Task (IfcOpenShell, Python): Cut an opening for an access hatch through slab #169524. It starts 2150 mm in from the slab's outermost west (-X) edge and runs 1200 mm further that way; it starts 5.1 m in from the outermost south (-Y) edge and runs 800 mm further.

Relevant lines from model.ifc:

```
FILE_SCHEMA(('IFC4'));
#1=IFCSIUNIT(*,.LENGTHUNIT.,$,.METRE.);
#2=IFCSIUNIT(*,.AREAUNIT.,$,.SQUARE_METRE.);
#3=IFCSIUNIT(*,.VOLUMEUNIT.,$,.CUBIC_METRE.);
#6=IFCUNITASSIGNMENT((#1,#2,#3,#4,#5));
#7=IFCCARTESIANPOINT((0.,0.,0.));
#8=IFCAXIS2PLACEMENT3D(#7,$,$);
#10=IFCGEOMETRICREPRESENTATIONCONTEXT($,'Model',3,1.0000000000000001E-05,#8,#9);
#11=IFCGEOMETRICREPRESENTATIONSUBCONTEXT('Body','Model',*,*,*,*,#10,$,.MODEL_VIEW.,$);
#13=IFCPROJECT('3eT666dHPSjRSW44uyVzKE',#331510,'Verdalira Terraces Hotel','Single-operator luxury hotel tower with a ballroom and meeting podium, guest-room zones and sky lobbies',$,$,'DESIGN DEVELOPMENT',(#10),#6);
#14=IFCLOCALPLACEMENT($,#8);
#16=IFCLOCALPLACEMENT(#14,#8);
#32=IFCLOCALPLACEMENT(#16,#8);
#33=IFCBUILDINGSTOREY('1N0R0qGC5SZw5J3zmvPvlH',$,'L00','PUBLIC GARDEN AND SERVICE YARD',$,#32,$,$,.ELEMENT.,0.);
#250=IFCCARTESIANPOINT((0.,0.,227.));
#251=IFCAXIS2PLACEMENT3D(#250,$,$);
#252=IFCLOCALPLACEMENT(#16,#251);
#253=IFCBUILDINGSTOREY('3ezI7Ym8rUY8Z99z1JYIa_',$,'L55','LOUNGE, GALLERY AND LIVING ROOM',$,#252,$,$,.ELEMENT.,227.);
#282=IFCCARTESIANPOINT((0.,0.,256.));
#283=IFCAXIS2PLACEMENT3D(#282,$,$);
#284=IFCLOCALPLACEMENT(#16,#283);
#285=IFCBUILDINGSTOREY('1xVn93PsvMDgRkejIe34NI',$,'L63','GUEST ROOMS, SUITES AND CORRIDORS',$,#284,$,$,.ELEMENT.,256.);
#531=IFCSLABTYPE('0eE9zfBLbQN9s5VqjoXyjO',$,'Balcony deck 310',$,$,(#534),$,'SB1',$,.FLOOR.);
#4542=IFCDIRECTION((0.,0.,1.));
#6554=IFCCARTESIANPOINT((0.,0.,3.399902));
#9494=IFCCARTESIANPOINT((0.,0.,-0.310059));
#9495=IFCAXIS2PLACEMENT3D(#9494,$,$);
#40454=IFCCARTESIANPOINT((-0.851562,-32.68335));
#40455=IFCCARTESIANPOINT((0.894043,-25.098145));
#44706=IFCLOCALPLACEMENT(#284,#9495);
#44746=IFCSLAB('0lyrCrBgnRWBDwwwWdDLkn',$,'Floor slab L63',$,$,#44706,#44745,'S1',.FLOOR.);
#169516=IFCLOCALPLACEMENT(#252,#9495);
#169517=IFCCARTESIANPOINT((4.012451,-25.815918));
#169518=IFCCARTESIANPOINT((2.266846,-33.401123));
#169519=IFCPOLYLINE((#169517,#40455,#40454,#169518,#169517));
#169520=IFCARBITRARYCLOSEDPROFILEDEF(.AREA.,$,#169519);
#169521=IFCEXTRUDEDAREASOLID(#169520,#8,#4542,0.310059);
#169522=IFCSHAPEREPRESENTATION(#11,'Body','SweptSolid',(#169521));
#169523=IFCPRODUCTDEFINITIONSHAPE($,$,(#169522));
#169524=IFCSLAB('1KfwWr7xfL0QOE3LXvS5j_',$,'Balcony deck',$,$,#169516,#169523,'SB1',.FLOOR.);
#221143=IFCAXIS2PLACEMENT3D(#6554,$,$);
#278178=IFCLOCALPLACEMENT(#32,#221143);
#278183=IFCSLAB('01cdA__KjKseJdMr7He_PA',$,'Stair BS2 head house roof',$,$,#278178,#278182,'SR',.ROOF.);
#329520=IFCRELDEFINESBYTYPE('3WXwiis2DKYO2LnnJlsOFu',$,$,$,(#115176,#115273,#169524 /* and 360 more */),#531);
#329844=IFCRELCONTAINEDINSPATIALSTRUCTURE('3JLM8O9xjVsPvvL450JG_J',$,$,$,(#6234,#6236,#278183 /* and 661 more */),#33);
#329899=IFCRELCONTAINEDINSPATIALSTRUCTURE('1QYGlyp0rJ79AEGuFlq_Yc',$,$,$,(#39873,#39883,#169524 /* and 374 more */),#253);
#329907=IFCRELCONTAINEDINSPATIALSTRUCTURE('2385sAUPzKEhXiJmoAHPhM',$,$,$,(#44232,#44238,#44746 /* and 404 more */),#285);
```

```python
import numpy as np
import ifcopenshell
import ifcopenshell.api.feature
import ifcopenshell.api.geometry
import ifcopenshell.api.root
import ifcopenshell.geom
import ifcopenshell.util.placement
import ifcopenshell.util.representation
import ifcopenshell.util.shape
import ifcopenshell.util.unit

model = ifcopenshell.open("model.ifc")
unit_scale = ifcopenshell.util.unit.calculate_unit_scale(model)
settings = ifcopenshell.geom.settings()


def volume(element):
    """Net volume in cubic metres, openings subtracted."""
    shape = ifcopenshell.geom.create_shape(settings, element)
    return ifcopenshell.util.shape.get_volume(shape.geometry)


slab = model.by_id(169524)
before = volume(slab)

# Extent in the slab's own axes, in metres. The edges named are its -X and -Y sides.
slab_shape = ifcopenshell.geom.create_shape(settings, slab)
vertices = ifcopenshell.util.shape.get_vertices(slab_shape.geometry)
x_min, y_min, bottom = vertices.min(axis=0)
top = vertices[:, 2].max()

opening = ifcopenshell.api.root.create_entity(model, ifc_class="IfcOpeningElement", name="Access hatch opening", predefined_type="OPENING")
context = ifcopenshell.util.representation.get_context(model, "Model", "Body", "MODEL_VIEW")
width, depth = 1.2, 0.8
outline = [(0.0, 0.0), (width, 0.0), (width, depth), (0.0, depth), (0.0, 0.0)]
# Overshoot both faces by 50 mm so the cut is clean.
shape = ifcopenshell.api.geometry.add_slab_representation(
    model, context=context, depth=top - bottom + 0.1, polyline=outline
)
ifcopenshell.api.geometry.assign_representation(model, product=opening, representation=shape)

matrix = ifcopenshell.util.placement.get_local_placement(slab.ObjectPlacement)
matrix[:, 3] = matrix @ np.append(np.array([x_min + 2.15, y_min + 5.1, bottom - 0.05]) / unit_scale, 1.0)
ifcopenshell.api.geometry.edit_object_placement(model, product=opening, matrix=matrix, is_si=False)
ifcopenshell.api.feature.add_feature(model, feature=opening, element=slab)

after = volume(slab)

print(f"slab volume {before:.3f} -> {after:.3f} m3")

model.write("model_rev.ifc")
```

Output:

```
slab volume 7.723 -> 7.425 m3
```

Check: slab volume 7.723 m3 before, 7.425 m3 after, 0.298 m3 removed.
